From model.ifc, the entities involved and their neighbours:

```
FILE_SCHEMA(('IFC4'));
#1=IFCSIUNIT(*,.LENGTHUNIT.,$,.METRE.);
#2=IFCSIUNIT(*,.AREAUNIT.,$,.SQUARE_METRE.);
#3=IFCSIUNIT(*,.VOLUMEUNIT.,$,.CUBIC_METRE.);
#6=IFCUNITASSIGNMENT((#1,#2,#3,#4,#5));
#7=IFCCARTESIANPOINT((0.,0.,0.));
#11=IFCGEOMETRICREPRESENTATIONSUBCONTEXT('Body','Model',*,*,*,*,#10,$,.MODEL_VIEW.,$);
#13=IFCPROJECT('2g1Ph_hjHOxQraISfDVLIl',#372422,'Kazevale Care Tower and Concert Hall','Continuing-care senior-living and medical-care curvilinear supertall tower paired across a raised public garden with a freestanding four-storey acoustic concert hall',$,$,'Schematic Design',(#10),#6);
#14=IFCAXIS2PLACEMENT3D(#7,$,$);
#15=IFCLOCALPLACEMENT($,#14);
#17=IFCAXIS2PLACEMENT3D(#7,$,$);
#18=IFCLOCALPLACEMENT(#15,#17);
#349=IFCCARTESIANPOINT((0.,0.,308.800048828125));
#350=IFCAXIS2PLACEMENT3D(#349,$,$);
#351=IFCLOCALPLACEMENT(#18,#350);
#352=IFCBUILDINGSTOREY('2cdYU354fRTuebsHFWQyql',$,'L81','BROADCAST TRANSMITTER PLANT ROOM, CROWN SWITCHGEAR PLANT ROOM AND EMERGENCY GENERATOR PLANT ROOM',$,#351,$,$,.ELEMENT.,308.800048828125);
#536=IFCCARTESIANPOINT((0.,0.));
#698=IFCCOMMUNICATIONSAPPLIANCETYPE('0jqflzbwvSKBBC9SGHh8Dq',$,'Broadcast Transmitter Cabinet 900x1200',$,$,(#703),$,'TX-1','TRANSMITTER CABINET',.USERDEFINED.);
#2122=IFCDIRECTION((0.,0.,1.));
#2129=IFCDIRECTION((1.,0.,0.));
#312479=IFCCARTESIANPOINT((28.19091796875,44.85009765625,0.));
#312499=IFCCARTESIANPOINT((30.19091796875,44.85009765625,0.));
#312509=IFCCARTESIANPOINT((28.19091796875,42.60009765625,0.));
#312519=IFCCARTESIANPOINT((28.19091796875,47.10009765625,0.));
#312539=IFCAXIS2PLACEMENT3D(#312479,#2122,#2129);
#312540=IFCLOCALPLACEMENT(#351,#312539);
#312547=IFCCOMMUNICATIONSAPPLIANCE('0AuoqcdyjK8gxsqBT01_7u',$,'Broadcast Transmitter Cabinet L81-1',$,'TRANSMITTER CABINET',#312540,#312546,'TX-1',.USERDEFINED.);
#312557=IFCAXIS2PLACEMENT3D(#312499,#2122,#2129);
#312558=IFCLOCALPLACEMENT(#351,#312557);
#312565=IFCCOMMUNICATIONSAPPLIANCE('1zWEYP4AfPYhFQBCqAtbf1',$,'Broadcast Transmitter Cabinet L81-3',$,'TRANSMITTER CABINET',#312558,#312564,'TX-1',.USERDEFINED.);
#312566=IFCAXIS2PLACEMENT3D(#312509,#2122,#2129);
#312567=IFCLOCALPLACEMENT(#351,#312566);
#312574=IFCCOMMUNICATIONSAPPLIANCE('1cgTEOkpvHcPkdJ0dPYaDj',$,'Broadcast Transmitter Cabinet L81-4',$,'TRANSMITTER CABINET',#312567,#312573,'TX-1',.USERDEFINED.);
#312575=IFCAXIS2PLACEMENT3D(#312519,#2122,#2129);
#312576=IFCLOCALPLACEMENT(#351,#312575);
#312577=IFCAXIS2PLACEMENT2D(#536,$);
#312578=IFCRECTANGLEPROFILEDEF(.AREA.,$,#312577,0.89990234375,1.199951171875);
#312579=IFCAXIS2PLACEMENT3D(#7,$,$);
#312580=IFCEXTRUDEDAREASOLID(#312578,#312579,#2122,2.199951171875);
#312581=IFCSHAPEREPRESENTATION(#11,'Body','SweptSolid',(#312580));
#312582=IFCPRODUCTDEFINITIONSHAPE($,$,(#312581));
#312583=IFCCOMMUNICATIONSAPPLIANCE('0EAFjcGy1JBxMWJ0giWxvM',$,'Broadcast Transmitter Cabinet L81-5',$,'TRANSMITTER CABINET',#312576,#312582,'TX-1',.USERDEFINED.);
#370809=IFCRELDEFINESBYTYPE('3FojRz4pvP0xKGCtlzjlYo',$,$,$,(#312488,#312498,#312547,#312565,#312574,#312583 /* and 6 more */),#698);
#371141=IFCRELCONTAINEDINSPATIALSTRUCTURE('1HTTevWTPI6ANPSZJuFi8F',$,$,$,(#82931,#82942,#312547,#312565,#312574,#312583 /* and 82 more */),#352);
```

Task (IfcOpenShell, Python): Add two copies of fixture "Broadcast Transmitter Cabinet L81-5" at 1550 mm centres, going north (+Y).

```python
import numpy as np
import ifcopenshell
import ifcopenshell.api.geometry
import ifcopenshell.api.root
import ifcopenshell.util.element
import ifcopenshell.util.placement

model = ifcopenshell.open("model.ifc")

source = model.by_guid("0EAFjcGy1JBxMWJ0giWxvM")
base = ifcopenshell.util.placement.get_local_placement(source.ObjectPlacement)
step = np.array([0.0, 1.0, 0.0]) * 1.55

for i in range(1, 3):
    copy = ifcopenshell.api.root.copy_class(model, product=source)
    copy.Representation = ifcopenshell.util.element.copy_deep(
        model, source.Representation, exclude=["IfcGeometricRepresentationContext", "IfcRepresentationMap"]
    )
    copy.Tag = None
    matrix = base.copy()
    matrix[:3, 3] += i * step
    print("added at", matrix[:3, 3].round(3) + 0.0)
    ifcopenshell.api.geometry.edit_object_placement(model, product=copy, matrix=matrix, is_si=False)

model.write("model_v2.ifc")
```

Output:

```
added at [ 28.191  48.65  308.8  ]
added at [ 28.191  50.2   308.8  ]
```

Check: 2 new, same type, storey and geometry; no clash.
